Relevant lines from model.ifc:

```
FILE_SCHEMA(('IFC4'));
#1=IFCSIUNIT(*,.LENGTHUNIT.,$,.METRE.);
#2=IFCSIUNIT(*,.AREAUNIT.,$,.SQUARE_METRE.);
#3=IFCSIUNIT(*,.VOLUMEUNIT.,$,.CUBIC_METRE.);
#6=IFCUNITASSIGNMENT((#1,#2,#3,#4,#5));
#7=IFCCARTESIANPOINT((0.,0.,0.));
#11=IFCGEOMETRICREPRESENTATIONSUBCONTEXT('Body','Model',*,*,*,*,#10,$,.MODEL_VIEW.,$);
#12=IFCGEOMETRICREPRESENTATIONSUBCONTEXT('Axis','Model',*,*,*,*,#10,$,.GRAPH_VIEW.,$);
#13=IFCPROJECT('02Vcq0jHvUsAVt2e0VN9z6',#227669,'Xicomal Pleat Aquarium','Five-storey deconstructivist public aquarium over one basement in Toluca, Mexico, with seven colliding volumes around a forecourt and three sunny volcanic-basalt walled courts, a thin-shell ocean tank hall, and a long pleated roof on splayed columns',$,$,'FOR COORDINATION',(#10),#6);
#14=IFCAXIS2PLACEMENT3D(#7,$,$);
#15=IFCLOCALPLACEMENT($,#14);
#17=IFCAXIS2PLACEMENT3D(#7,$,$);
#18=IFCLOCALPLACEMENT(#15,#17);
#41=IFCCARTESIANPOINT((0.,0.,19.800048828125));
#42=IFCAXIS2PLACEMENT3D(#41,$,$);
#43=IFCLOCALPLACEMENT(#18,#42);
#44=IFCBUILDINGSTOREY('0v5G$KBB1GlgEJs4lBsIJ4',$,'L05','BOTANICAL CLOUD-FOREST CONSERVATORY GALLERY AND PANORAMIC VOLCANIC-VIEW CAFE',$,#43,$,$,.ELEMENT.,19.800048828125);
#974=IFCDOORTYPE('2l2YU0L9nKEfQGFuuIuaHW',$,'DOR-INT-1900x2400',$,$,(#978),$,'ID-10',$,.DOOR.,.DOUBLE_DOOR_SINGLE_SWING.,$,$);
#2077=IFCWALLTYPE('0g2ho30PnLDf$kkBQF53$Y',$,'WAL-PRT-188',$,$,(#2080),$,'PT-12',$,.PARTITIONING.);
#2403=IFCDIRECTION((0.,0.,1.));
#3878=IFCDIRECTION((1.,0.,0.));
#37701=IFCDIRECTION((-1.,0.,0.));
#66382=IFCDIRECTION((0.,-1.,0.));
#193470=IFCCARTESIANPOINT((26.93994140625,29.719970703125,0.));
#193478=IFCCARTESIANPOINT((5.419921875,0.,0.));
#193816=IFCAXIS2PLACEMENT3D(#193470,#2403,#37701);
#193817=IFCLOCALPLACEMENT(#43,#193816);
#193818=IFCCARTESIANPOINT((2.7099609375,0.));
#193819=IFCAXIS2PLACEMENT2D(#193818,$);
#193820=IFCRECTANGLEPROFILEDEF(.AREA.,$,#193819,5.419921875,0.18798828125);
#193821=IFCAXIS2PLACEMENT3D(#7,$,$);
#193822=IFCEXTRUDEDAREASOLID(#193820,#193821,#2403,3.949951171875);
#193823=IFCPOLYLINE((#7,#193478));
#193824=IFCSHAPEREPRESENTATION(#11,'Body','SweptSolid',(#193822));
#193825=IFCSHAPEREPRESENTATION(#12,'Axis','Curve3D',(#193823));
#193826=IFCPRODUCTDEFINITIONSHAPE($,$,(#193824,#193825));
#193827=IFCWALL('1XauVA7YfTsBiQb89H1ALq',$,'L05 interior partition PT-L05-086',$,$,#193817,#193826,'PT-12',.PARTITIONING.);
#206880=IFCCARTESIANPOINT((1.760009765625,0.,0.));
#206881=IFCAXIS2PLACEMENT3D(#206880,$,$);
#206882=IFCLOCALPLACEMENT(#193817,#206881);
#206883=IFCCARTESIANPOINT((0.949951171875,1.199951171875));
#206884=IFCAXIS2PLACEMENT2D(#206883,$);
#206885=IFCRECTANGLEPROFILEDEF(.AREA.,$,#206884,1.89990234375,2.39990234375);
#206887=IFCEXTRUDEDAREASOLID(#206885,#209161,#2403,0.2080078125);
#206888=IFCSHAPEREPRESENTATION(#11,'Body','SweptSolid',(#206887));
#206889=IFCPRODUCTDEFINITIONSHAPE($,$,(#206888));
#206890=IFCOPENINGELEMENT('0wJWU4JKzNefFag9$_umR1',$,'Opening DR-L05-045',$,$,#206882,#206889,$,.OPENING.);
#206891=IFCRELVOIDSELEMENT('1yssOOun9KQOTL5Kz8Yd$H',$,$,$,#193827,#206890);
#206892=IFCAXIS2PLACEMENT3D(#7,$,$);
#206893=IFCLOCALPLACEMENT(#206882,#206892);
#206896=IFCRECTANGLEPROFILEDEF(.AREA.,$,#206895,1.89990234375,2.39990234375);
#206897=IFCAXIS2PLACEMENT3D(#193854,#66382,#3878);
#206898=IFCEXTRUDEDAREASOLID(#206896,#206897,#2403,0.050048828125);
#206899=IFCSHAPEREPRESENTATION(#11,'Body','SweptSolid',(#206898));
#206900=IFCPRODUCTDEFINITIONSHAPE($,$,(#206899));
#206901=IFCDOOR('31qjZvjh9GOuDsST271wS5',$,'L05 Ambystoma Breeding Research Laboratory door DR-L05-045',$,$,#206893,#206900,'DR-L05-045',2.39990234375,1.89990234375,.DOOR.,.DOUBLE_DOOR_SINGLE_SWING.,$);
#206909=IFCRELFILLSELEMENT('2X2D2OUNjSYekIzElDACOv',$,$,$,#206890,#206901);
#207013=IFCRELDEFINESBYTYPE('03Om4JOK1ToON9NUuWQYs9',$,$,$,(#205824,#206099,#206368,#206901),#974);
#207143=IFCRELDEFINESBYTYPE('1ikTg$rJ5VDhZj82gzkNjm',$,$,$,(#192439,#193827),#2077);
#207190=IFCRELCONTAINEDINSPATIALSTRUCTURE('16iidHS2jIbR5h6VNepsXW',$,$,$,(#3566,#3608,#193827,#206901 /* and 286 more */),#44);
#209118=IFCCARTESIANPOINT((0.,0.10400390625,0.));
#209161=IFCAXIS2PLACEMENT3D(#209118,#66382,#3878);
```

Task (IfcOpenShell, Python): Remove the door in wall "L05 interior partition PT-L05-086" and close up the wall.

```python
import ifcopenshell
import ifcopenshell.api.feature
import ifcopenshell.api.root
import ifcopenshell.geom
import ifcopenshell.util.shape

model = ifcopenshell.open("model.ifc")
settings = ifcopenshell.geom.settings()


def volume(element):
    """Net volume in cubic metres, openings subtracted."""
    shape = ifcopenshell.geom.create_shape(settings, element)
    return ifcopenshell.util.shape.get_volume(shape.geometry)


door = model.by_guid("31qjZvjh9GOuDsST271wS5")
opening = door.FillsVoids[0].RelatingOpeningElement
wall = opening.VoidsElements[0].RelatingBuildingElement
before = volume(wall)

ifcopenshell.api.root.remove_product(model, product=door)
ifcopenshell.api.feature.remove_feature(model, feature=opening)

after = volume(wall)

print(f"wall volume {before:.3f} -> {after:.3f} m3")

model.write("model_rev.ifc")
```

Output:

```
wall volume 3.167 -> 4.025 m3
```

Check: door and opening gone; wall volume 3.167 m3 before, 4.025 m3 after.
